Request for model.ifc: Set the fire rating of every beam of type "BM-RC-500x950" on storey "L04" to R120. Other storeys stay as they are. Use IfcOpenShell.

First a look at what the model holds.

```python
import ifcopenshell
import ifcopenshell.util.element

model = ifcopenshell.open("model.ifc")
print(model.schema)
storey = next(s for s in model.by_type("IfcBuildingStorey") if s.Name == "L04")
beams = [e for e in ifcopenshell.util.element.get_decomposition(storey) if e.is_a("IfcBeam")]
seen = {}
for e in beams:
    element_type = ifcopenshell.util.element.get_type(e)
    key = (element_type.Name if element_type != e and element_type else None, ifcopenshell.util.element.get_pset(e, "Pset_BeamCommon", "FireRating"))
    seen[key] = seen.get(key, 0) + 1
for (name, value), count in sorted(seen.items(), key=str):
    print(count, "x", name, "|", value)
```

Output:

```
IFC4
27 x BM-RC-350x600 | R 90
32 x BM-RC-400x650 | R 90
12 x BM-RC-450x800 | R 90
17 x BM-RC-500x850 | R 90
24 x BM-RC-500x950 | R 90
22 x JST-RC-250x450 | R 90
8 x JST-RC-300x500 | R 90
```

```python
import ifcopenshell
import ifcopenshell.api.pset
import ifcopenshell.util.element

model = ifcopenshell.open("model.ifc")

storey = next(s for s in model.by_type("IfcBuildingStorey") if s.Name == "L04")
beams = [e for e in ifcopenshell.util.element.get_decomposition(storey) if e.is_a("IfcBeam")]

count = 0
for e in beams:
    element_type = ifcopenshell.util.element.get_type(e)
    if element_type in (None, e) or element_type.Name != "BM-RC-500x950":
        continue
    # add_pset returns the element's existing set when there is one.
    pset = ifcopenshell.api.pset.add_pset(model, product=e, name="Pset_BeamCommon")
    ifcopenshell.api.pset.edit_pset(model, pset=pset, properties={"FireRating": "R120"})
    count += 1

print(count, "beams updated")

model.write("model-out.ifc")
```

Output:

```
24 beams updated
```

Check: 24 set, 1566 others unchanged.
